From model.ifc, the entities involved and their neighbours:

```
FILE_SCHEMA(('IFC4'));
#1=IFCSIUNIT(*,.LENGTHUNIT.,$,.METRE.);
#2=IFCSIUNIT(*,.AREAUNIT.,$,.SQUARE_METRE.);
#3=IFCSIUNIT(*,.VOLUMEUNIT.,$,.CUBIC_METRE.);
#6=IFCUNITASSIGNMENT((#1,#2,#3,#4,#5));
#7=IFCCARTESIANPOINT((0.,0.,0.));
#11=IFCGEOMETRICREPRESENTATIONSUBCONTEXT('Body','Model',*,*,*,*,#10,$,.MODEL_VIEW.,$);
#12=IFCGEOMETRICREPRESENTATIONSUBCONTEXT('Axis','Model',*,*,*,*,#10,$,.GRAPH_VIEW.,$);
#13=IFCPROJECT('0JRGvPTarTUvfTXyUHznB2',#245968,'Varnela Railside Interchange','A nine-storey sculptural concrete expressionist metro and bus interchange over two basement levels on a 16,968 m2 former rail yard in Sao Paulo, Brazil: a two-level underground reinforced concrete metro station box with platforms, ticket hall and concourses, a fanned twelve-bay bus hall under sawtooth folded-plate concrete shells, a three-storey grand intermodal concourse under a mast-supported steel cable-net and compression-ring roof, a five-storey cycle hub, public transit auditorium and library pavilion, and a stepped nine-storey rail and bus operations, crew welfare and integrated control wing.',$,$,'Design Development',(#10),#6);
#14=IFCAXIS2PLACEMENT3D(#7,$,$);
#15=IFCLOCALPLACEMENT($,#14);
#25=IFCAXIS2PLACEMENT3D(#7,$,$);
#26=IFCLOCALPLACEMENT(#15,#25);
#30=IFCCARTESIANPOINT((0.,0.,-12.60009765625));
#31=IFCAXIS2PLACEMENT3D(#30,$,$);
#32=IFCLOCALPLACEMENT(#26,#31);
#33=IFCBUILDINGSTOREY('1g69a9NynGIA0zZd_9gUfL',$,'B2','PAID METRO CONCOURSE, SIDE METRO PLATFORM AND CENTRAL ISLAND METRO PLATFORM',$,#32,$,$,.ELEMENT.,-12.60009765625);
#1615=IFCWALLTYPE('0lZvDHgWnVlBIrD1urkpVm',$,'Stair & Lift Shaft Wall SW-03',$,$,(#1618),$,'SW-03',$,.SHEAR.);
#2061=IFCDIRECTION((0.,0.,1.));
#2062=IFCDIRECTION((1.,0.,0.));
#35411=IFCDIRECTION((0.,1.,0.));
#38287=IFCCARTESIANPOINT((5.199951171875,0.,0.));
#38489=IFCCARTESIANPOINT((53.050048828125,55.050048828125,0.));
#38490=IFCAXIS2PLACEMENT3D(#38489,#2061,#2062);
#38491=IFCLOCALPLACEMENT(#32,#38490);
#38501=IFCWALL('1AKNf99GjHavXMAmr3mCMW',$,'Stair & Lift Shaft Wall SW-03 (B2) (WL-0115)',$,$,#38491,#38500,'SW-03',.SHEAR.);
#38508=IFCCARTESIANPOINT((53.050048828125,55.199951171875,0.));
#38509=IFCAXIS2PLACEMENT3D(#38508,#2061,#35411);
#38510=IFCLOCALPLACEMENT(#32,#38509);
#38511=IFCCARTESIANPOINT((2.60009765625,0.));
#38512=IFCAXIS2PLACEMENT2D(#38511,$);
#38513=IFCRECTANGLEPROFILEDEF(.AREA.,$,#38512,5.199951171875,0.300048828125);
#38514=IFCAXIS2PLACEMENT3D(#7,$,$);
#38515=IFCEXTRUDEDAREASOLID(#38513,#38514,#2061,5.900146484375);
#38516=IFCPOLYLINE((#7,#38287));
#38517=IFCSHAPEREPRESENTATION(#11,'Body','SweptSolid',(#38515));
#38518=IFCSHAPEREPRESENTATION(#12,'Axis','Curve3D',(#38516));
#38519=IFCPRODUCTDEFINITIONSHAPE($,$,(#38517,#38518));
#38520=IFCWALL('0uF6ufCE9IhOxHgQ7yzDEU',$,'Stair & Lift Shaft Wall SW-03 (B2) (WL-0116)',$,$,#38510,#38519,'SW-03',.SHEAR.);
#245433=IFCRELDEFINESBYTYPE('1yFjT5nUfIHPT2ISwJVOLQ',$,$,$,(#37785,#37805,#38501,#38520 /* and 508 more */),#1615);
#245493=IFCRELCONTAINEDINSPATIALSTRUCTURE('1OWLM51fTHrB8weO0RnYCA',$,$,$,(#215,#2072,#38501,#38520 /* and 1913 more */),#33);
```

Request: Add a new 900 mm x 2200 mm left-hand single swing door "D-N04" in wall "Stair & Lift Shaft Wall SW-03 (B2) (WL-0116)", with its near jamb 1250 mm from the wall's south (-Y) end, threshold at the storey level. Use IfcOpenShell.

```python
import numpy as np
import ifcopenshell
import ifcopenshell.api.feature
import ifcopenshell.api.geometry
import ifcopenshell.api.root
import ifcopenshell.api.spatial
import ifcopenshell.geom
import ifcopenshell.util.element
import ifcopenshell.util.placement
import ifcopenshell.util.representation
import ifcopenshell.util.shape
import ifcopenshell.util.unit

model = ifcopenshell.open("model.ifc")
unit_scale = ifcopenshell.util.unit.calculate_unit_scale(model)
settings = ifcopenshell.geom.settings()


def volume(element):
    """Net volume in cubic metres, openings subtracted."""
    shape = ifcopenshell.geom.create_shape(settings, element)
    return ifcopenshell.util.shape.get_volume(shape.geometry)


wall = model.by_guid("0uF6ufCE9IhOxHgQ7yzDEU")
storey = ifcopenshell.util.element.get_container(wall, ifc_class="IfcBuildingStorey")
context = ifcopenshell.util.representation.get_context(model, "Model", "Body", "MODEL_VIEW")
before = volume(wall)

width, height, from_end, sill = 0.9, 2.2, 1.25, 0.0  # metres

# The wall runs along its own X axis, and the end named is its -X end.
wall_shape = ifcopenshell.geom.create_shape(settings, wall)
x, y, z = ifcopenshell.util.shape.get_vertices(wall_shape.geometry).T
start = x.min() + from_end
face, thickness = float(y.min()), float(y.max() - y.min())
wall_matrix = ifcopenshell.util.placement.get_local_placement(wall.ObjectPlacement)
level = ifcopenshell.util.placement.get_local_placement(storey.ObjectPlacement)[2, 3]


def in_wall(x, y):
    """Placement at x, y metres in the wall's axes, at sill height."""
    matrix = wall_matrix.copy()
    matrix[:, 3] = wall_matrix @ np.array([x / unit_scale, y / unit_scale, 0.0, 1.0])
    matrix[2, 3] = level + sill / unit_scale
    return matrix


# Opening: a box that overshoots both wall faces by 50 mm.
opening = ifcopenshell.api.root.create_entity(model, ifc_class="IfcOpeningElement", predefined_type="OPENING")
box = ifcopenshell.api.geometry.add_wall_representation(
    model, context=context, length=width, height=height, thickness=thickness + 0.1
)
ifcopenshell.api.geometry.assign_representation(model, product=opening, representation=box)
ifcopenshell.api.geometry.edit_object_placement(model, product=opening, matrix=in_wall(start, face - 0.05), is_si=False)
ifcopenshell.api.feature.add_feature(model, feature=opening, element=wall)

door = ifcopenshell.api.root.create_entity(model, ifc_class="IfcDoor", name="D-N04", predefined_type="DOOR")
door.OverallWidth, door.OverallHeight = width / unit_scale, height / unit_scale
door.OperationType = "SINGLE_SWING_LEFT"
body = ifcopenshell.api.geometry.add_door_representation(
    model,
    context=context,
    overall_width=door.OverallWidth,
    overall_height=door.OverallHeight,
    operation_type="SINGLE_SWING_LEFT",
    lining_properties={"LiningDepth": thickness / unit_scale, "ThresholdDepth": thickness / unit_scale},
)
ifcopenshell.api.geometry.assign_representation(model, product=door, representation=body)
ifcopenshell.api.spatial.assign_container(model, products=[door], relating_structure=storey)
ifcopenshell.api.feature.add_filling(model, opening=opening, element=door)

# The lining spans the wall, so the door starts at the wall face.
ifcopenshell.api.geometry.edit_object_placement(model, product=door, matrix=in_wall(start, face), is_si=False)

after = volume(wall)

print(f"wall volume {before:.3f} -> {after:.3f} m3")

model.write("model_updated.ifc")
```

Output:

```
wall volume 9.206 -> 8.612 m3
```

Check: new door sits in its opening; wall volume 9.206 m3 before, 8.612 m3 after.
